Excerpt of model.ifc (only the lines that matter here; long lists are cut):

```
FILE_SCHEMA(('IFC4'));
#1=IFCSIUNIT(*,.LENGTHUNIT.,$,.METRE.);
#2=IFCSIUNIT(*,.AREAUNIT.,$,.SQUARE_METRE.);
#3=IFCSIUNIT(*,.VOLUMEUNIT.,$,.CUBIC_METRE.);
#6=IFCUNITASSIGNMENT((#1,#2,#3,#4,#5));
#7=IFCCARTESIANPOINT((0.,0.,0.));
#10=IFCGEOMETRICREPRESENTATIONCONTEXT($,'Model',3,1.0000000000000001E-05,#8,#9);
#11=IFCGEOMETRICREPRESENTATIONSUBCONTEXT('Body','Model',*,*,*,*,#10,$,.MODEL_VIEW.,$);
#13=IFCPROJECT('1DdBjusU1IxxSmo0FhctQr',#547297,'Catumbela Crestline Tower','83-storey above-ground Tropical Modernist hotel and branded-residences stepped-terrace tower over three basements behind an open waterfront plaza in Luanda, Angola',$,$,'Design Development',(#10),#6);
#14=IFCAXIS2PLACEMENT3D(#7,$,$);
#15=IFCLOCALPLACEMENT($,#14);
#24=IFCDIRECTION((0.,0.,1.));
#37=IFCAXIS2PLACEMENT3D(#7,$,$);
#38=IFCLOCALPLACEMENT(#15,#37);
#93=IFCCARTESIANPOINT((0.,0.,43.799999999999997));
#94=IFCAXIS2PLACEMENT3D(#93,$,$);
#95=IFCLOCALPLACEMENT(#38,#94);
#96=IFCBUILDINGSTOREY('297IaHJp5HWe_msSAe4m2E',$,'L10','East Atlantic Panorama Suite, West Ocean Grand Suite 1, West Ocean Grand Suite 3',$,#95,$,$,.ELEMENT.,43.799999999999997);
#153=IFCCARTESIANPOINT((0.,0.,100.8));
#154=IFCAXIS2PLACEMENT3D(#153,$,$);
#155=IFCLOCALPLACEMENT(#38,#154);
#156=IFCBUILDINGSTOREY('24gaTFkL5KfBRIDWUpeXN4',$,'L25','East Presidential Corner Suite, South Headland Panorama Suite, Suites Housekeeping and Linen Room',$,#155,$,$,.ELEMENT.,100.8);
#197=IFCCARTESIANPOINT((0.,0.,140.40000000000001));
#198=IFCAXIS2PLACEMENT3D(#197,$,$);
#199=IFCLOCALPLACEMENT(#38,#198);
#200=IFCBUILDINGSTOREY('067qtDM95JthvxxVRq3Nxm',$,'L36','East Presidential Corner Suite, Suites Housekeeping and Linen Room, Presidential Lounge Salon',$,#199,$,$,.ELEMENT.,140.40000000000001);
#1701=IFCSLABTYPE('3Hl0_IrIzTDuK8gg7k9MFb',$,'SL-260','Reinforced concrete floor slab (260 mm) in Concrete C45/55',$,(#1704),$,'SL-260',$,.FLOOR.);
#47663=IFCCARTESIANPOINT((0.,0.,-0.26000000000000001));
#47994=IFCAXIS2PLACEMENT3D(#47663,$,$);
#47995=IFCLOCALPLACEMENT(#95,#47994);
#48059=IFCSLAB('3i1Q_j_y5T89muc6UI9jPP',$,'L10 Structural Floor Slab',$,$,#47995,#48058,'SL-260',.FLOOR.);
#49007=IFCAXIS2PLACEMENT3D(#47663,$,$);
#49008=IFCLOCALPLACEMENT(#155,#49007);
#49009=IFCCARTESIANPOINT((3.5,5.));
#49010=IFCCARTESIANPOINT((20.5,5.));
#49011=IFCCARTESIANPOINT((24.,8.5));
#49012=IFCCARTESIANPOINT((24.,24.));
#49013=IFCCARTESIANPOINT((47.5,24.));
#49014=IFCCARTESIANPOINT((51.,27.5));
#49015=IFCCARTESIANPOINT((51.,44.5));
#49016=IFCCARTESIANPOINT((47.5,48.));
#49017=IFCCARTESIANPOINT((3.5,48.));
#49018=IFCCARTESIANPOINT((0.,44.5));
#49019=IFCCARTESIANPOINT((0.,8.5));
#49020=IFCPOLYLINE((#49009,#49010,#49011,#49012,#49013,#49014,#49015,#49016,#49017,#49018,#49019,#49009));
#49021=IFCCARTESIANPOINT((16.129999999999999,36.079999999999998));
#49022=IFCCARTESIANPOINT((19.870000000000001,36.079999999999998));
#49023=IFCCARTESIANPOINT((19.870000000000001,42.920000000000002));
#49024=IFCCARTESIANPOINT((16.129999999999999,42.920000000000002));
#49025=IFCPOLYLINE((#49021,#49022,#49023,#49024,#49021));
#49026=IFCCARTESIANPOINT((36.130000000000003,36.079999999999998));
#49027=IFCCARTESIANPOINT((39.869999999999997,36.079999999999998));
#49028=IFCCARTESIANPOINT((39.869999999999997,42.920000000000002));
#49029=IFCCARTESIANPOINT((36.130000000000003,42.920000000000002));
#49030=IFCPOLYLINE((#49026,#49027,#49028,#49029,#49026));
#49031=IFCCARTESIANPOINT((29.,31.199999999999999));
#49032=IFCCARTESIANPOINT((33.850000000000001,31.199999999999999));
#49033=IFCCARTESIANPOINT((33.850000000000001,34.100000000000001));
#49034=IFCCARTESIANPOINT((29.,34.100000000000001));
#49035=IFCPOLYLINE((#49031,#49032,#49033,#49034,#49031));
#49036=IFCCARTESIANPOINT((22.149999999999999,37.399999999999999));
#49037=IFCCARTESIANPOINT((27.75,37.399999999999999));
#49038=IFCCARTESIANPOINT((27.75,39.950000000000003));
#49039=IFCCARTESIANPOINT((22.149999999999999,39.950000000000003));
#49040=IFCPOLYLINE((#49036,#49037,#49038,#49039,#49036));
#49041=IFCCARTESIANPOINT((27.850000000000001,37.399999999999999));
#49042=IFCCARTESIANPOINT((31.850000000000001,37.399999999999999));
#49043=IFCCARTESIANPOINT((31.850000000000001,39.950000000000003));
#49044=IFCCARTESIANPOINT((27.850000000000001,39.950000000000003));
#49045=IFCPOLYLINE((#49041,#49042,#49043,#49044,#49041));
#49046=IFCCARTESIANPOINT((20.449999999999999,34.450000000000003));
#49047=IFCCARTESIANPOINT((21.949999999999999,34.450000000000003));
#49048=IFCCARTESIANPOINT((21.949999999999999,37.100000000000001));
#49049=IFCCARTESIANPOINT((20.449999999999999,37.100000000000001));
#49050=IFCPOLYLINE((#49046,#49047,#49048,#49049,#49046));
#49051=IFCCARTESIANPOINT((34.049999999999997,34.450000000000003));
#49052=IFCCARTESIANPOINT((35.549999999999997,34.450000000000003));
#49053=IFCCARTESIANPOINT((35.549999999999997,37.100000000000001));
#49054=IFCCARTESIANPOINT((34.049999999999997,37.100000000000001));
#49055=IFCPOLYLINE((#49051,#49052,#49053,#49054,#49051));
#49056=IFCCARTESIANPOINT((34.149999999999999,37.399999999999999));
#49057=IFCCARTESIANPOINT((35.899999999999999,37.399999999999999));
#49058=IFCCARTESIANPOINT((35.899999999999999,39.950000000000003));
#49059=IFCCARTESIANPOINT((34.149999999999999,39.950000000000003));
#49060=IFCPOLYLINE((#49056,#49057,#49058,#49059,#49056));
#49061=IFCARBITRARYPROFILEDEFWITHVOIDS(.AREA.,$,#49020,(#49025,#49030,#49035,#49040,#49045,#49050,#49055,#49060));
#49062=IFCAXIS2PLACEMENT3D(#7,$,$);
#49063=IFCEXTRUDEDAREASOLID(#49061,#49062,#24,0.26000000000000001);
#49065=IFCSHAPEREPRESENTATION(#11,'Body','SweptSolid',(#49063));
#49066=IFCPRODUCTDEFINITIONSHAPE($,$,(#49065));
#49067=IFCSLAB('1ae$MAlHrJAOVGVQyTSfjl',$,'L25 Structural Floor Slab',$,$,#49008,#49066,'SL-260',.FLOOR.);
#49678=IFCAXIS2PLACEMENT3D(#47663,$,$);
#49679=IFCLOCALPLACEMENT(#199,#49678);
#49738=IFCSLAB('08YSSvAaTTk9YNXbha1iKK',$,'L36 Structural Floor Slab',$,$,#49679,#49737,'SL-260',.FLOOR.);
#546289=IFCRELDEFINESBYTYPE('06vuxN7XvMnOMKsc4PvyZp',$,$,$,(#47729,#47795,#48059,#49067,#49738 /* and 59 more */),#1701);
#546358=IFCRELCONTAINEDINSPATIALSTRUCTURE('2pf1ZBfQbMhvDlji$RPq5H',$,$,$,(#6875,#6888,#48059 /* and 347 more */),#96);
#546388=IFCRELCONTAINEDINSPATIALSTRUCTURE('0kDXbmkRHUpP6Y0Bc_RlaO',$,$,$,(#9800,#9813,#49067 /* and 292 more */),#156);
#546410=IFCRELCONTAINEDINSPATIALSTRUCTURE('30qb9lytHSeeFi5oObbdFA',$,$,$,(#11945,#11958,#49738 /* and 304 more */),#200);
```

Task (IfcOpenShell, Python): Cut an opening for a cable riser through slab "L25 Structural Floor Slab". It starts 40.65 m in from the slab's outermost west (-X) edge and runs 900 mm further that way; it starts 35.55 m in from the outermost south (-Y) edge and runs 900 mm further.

```python
import numpy as np
import ifcopenshell
import ifcopenshell.api.feature
import ifcopenshell.api.geometry
import ifcopenshell.api.root
import ifcopenshell.geom
import ifcopenshell.util.placement
import ifcopenshell.util.representation
import ifcopenshell.util.shape
import ifcopenshell.util.unit

model = ifcopenshell.open("model.ifc")
unit_scale = ifcopenshell.util.unit.calculate_unit_scale(model)
settings = ifcopenshell.geom.settings()


def volume(element):
    """Net volume in cubic metres, openings subtracted."""
    shape = ifcopenshell.geom.create_shape(settings, element)
    return ifcopenshell.util.shape.get_volume(shape.geometry)


slab = model.by_id(49067)
before = volume(slab)

# Extent in the slab's own axes, in metres. The edges named are its -X and -Y sides.
slab_shape = ifcopenshell.geom.create_shape(settings, slab)
vertices = ifcopenshell.util.shape.get_vertices(slab_shape.geometry)
x_min, y_min, bottom = vertices.min(axis=0)
top = vertices[:, 2].max()

opening = ifcopenshell.api.root.create_entity(model, ifc_class="IfcOpeningElement", name="Cable riser opening", predefined_type="OPENING")
context = ifcopenshell.util.representation.get_context(model, "Model", "Body", "MODEL_VIEW")
width, depth = 0.9, 0.9
outline = [(0.0, 0.0), (width, 0.0), (width, depth), (0.0, depth), (0.0, 0.0)]
# Overshoot both faces by 50 mm so the cut is clean.
shape = ifcopenshell.api.geometry.add_slab_representation(
    model, context=context, depth=top - bottom + 0.1, polyline=outline
)
ifcopenshell.api.geometry.assign_representation(model, product=opening, representation=shape)

matrix = ifcopenshell.util.placement.get_local_placement(slab.ObjectPlacement)
matrix[:, 3] = matrix @ np.append(np.array([x_min + 40.65, y_min + 35.55, bottom - 0.05]) / unit_scale, 1.0)
ifcopenshell.api.geometry.edit_object_placement(model, product=opening, matrix=matrix, is_si=False)
ifcopenshell.api.feature.add_feature(model, feature=opening, element=slab)

after = volume(slab)

print(f"slab volume {before:.3f} -> {after:.3f} m3")

model.write("model_updated.ifc")
```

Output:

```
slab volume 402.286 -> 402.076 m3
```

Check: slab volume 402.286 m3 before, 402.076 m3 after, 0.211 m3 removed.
